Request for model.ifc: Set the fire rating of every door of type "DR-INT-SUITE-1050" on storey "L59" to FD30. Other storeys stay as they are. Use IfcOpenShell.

First a look at what the model holds.

```python
import ifcopenshell
import ifcopenshell.util.element

model = ifcopenshell.open("model.ifc")
print(model.schema)
storey = next(s for s in model.by_type("IfcBuildingStorey") if s.Name == "L59")
doors = [e for e in ifcopenshell.util.element.get_decomposition(storey) if e.is_a("IfcDoor")]
seen = {}
for e in doors:
    element_type = ifcopenshell.util.element.get_type(e)
    key = (element_type.Name if element_type != e and element_type else None, ifcopenshell.util.element.get_pset(e, "Pset_DoorCommon", "FireRating"))
    seen[key] = seen.get(key, 0) + 1
for (name, value), count in sorted(seen.items(), key=str):
    print(count, "x", name, "|", value)
```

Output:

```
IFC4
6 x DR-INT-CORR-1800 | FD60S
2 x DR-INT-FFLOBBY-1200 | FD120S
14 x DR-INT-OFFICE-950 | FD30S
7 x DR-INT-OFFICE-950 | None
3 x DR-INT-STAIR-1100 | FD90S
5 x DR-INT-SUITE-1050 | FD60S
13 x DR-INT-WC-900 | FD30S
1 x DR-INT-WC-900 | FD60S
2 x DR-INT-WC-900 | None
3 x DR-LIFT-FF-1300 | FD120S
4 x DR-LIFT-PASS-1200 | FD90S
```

```python
import ifcopenshell
import ifcopenshell.api.pset
import ifcopenshell.util.element

model = ifcopenshell.open("model.ifc")

storey = next(s for s in model.by_type("IfcBuildingStorey") if s.Name == "L59")
doors = [e for e in ifcopenshell.util.element.get_decomposition(storey) if e.is_a("IfcDoor")]

count = 0
for e in doors:
    element_type = ifcopenshell.util.element.get_type(e)
    if element_type in (None, e) or element_type.Name != "DR-INT-SUITE-1050":
        continue
    found = ifcopenshell.util.element.get_pset(e, "Pset_DoorCommon", should_inherit=False)
    if found:
        pset = model.by_id(found["id"])
        if len(ifcopenshell.util.element.get_elements_by_pset(pset)) > 1:
            pset = ifcopenshell.api.pset.unshare_pset(model, products=[e], pset=pset)[0]
    else:
        pset = ifcopenshell.api.pset.add_pset(model, product=e, name="Pset_DoorCommon")
    ifcopenshell.api.pset.edit_pset(model, pset=pset, properties={"FireRating": "FD30"})
    count += 1

print(count, "doors updated")

model.write("model_updated.ifc")
```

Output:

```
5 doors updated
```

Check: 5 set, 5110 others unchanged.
